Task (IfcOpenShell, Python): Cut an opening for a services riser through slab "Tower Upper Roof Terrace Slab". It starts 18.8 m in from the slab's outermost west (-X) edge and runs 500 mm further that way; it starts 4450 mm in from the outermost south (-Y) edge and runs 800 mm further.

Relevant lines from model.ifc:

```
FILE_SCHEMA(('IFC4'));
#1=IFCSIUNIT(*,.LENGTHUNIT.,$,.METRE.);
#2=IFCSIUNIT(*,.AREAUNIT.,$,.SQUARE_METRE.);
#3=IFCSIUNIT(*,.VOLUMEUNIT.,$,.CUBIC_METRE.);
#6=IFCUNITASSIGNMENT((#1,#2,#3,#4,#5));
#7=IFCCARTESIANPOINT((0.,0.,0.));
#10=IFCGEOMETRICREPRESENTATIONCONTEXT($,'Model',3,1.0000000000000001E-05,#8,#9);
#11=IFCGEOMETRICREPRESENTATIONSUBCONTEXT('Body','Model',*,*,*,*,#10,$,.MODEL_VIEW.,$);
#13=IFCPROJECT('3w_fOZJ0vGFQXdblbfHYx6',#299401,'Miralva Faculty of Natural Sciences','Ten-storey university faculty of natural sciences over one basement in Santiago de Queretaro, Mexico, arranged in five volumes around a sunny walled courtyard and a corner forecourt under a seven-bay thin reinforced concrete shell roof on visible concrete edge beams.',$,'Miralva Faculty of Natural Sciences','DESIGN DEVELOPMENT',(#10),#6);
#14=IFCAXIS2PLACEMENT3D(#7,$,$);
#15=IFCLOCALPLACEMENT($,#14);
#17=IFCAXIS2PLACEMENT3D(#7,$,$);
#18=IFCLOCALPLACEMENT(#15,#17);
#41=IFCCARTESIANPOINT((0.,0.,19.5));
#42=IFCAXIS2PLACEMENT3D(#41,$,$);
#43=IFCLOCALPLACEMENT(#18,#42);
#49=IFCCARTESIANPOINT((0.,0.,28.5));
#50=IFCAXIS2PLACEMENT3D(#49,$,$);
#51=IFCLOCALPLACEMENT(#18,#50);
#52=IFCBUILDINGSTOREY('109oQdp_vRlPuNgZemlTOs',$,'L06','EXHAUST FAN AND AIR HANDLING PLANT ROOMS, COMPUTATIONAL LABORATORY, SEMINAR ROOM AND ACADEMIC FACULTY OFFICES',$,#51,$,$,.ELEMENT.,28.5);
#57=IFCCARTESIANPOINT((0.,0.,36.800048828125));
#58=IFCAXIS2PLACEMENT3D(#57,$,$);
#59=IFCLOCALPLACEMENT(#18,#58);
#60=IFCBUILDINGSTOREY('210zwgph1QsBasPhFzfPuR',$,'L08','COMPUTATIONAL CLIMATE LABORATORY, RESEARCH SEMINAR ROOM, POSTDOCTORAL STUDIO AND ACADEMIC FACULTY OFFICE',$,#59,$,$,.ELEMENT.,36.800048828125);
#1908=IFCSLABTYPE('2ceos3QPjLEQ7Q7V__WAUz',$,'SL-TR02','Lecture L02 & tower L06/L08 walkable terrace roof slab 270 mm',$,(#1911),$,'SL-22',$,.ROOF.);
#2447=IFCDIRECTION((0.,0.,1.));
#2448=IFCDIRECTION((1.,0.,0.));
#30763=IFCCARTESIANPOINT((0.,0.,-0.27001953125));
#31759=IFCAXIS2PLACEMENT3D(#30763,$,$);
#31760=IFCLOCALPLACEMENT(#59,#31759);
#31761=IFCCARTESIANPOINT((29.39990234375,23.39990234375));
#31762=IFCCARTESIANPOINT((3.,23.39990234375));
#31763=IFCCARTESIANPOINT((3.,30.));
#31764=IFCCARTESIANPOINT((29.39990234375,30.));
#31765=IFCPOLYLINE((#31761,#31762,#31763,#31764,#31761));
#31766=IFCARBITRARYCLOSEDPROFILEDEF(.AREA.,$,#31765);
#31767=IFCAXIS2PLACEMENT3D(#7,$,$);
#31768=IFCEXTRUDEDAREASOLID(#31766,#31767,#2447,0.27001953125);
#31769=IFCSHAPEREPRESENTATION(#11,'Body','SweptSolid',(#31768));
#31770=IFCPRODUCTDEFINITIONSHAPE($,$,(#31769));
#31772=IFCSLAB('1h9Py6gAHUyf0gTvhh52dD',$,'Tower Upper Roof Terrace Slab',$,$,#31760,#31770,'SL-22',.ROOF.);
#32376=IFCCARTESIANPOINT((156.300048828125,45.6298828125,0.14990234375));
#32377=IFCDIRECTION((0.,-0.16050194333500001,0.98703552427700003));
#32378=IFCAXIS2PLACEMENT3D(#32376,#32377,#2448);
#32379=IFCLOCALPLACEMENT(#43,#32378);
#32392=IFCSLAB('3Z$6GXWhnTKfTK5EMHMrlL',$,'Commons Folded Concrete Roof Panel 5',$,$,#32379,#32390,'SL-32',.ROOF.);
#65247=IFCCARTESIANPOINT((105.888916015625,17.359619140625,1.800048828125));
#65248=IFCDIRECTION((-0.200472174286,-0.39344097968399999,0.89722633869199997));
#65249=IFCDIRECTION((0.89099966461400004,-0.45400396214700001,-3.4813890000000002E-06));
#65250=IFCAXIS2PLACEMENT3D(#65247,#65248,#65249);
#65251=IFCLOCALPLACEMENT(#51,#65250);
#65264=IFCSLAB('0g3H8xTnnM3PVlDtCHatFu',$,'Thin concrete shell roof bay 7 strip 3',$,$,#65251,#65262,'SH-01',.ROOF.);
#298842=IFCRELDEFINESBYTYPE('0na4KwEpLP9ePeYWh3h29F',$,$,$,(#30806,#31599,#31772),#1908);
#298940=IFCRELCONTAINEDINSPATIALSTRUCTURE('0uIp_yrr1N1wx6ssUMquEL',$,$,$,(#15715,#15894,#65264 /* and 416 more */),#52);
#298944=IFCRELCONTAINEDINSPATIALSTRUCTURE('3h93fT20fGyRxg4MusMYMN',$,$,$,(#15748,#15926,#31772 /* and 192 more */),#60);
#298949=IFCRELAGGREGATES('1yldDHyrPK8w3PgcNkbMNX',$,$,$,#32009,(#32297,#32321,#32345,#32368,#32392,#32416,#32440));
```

```python
import numpy as np
import ifcopenshell
import ifcopenshell.api.feature
import ifcopenshell.api.geometry
import ifcopenshell.api.root
import ifcopenshell.geom
import ifcopenshell.util.placement
import ifcopenshell.util.representation
import ifcopenshell.util.shape
import ifcopenshell.util.unit

model = ifcopenshell.open("model.ifc")
unit_scale = ifcopenshell.util.unit.calculate_unit_scale(model)
settings = ifcopenshell.geom.settings()


def volume(element):
    """Net volume in cubic metres, openings subtracted."""
    shape = ifcopenshell.geom.create_shape(settings, element)
    return ifcopenshell.util.shape.get_volume(shape.geometry)


slab = model.by_id(31772)
before = volume(slab)

# Extent in the slab's own axes, in metres. The edges named are its -X and -Y sides.
slab_shape = ifcopenshell.geom.create_shape(settings, slab)
vertices = ifcopenshell.util.shape.get_vertices(slab_shape.geometry)
x_min, y_min, bottom = vertices.min(axis=0)
top = vertices[:, 2].max()

opening = ifcopenshell.api.root.create_entity(model, ifc_class="IfcOpeningElement", name="Services riser opening", predefined_type="OPENING")
context = ifcopenshell.util.representation.get_context(model, "Model", "Body", "MODEL_VIEW")
width, depth = 0.5, 0.8
outline = [(0.0, 0.0), (width, 0.0), (width, depth), (0.0, depth), (0.0, 0.0)]
# Overshoot both faces by 50 mm so the cut is clean.
shape = ifcopenshell.api.geometry.add_slab_representation(
    model, context=context, depth=top - bottom + 0.1, polyline=outline
)
ifcopenshell.api.geometry.assign_representation(model, product=opening, representation=shape)

matrix = ifcopenshell.util.placement.get_local_placement(slab.ObjectPlacement)
matrix[:, 3] = matrix @ np.append(np.array([x_min + 18.8, y_min + 4.45, bottom - 0.05]) / unit_scale, 1.0)
ifcopenshell.api.geometry.edit_object_placement(model, product=opening, matrix=matrix, is_si=False)
ifcopenshell.api.feature.add_feature(model, feature=opening, element=slab)

after = volume(slab)

print(f"slab volume {before:.3f} -> {after:.3f} m3")

model.write("model-out.ifc")
```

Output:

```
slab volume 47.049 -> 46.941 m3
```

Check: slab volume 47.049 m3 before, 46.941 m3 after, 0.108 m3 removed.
